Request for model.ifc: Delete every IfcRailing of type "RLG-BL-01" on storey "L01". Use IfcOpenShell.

First a look at what the model holds.

```python
import ifcopenshell
import ifcopenshell.util.element

model = ifcopenshell.open("model.ifc")
print(model.schema)
storey = next(s for s in model.by_type("IfcBuildingStorey") if s.Name == "L01")
railings = [e for e in ifcopenshell.util.element.get_decomposition(storey) if e.is_a("IfcRailing")]
seen = {}
for e in railings:
    element_type = ifcopenshell.util.element.get_type(e)
    name = element_type.Name if element_type not in (None, e) else None
    seen[name] = seen.get(name, 0) + 1
for name, count in sorted(seen.items(), key=str):
    print(count, "x", name)
```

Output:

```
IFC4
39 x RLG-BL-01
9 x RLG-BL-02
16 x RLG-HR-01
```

```python
import ifcopenshell
import ifcopenshell.api.root
import ifcopenshell.util.element

model = ifcopenshell.open("model.ifc")

storey = next(s for s in model.by_type("IfcBuildingStorey") if s.Name == "L01")
railings = [e for e in ifcopenshell.util.element.get_decomposition(storey) if e.is_a("IfcRailing")]
targets = [e for e in railings if (t := ifcopenshell.util.element.get_type(e)) not in (None, e) and t.Name == "RLG-BL-01"]

for e in targets:
    ifcopenshell.api.root.remove_product(model, product=e)
print(len(targets), "removed")

model.write("model_edited.ifc")
```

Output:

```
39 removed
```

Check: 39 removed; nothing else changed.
